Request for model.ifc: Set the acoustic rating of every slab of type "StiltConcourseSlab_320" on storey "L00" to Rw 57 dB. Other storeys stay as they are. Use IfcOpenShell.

First a look at what the model holds.

```python
import ifcopenshell
import ifcopenshell.util.element

model = ifcopenshell.open("model.ifc")
print(model.schema)
storey = next(s for s in model.by_type("IfcBuildingStorey") if s.Name == "L00")
slabs = [e for e in ifcopenshell.util.element.get_decomposition(storey) if e.is_a("IfcSlab")]
seen = {}
for e in slabs:
    element_type = ifcopenshell.util.element.get_type(e)
    key = (element_type.Name if element_type != e and element_type else None, ifcopenshell.util.element.get_pset(e, "Pset_SlabCommon", "AcousticRating"))
    seen[key] = seen.get(key, 0) + 1
for (name, value), count in sorted(seen.items(), key=str):
    print(count, "x", name, "|", value)
```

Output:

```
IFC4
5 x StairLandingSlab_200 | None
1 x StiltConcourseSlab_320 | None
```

```python
import ifcopenshell
import ifcopenshell.api.pset
import ifcopenshell.util.element

model = ifcopenshell.open("model.ifc")

storey = next(s for s in model.by_type("IfcBuildingStorey") if s.Name == "L00")
slabs = [e for e in ifcopenshell.util.element.get_decomposition(storey) if e.is_a("IfcSlab")]

count = 0
for e in slabs:
    element_type = ifcopenshell.util.element.get_type(e)
    if element_type in (None, e) or element_type.Name != "StiltConcourseSlab_320":
        continue
    # add_pset returns the element's existing set when there is one.
    pset = ifcopenshell.api.pset.add_pset(model, product=e, name="Pset_SlabCommon")
    ifcopenshell.api.pset.edit_pset(model, pset=pset, properties={"AcousticRating": "Rw 57 dB"})
    count += 1

print(count, "slabs updated")

model.write("model_v2.ifc")
```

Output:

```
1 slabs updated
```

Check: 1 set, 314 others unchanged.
